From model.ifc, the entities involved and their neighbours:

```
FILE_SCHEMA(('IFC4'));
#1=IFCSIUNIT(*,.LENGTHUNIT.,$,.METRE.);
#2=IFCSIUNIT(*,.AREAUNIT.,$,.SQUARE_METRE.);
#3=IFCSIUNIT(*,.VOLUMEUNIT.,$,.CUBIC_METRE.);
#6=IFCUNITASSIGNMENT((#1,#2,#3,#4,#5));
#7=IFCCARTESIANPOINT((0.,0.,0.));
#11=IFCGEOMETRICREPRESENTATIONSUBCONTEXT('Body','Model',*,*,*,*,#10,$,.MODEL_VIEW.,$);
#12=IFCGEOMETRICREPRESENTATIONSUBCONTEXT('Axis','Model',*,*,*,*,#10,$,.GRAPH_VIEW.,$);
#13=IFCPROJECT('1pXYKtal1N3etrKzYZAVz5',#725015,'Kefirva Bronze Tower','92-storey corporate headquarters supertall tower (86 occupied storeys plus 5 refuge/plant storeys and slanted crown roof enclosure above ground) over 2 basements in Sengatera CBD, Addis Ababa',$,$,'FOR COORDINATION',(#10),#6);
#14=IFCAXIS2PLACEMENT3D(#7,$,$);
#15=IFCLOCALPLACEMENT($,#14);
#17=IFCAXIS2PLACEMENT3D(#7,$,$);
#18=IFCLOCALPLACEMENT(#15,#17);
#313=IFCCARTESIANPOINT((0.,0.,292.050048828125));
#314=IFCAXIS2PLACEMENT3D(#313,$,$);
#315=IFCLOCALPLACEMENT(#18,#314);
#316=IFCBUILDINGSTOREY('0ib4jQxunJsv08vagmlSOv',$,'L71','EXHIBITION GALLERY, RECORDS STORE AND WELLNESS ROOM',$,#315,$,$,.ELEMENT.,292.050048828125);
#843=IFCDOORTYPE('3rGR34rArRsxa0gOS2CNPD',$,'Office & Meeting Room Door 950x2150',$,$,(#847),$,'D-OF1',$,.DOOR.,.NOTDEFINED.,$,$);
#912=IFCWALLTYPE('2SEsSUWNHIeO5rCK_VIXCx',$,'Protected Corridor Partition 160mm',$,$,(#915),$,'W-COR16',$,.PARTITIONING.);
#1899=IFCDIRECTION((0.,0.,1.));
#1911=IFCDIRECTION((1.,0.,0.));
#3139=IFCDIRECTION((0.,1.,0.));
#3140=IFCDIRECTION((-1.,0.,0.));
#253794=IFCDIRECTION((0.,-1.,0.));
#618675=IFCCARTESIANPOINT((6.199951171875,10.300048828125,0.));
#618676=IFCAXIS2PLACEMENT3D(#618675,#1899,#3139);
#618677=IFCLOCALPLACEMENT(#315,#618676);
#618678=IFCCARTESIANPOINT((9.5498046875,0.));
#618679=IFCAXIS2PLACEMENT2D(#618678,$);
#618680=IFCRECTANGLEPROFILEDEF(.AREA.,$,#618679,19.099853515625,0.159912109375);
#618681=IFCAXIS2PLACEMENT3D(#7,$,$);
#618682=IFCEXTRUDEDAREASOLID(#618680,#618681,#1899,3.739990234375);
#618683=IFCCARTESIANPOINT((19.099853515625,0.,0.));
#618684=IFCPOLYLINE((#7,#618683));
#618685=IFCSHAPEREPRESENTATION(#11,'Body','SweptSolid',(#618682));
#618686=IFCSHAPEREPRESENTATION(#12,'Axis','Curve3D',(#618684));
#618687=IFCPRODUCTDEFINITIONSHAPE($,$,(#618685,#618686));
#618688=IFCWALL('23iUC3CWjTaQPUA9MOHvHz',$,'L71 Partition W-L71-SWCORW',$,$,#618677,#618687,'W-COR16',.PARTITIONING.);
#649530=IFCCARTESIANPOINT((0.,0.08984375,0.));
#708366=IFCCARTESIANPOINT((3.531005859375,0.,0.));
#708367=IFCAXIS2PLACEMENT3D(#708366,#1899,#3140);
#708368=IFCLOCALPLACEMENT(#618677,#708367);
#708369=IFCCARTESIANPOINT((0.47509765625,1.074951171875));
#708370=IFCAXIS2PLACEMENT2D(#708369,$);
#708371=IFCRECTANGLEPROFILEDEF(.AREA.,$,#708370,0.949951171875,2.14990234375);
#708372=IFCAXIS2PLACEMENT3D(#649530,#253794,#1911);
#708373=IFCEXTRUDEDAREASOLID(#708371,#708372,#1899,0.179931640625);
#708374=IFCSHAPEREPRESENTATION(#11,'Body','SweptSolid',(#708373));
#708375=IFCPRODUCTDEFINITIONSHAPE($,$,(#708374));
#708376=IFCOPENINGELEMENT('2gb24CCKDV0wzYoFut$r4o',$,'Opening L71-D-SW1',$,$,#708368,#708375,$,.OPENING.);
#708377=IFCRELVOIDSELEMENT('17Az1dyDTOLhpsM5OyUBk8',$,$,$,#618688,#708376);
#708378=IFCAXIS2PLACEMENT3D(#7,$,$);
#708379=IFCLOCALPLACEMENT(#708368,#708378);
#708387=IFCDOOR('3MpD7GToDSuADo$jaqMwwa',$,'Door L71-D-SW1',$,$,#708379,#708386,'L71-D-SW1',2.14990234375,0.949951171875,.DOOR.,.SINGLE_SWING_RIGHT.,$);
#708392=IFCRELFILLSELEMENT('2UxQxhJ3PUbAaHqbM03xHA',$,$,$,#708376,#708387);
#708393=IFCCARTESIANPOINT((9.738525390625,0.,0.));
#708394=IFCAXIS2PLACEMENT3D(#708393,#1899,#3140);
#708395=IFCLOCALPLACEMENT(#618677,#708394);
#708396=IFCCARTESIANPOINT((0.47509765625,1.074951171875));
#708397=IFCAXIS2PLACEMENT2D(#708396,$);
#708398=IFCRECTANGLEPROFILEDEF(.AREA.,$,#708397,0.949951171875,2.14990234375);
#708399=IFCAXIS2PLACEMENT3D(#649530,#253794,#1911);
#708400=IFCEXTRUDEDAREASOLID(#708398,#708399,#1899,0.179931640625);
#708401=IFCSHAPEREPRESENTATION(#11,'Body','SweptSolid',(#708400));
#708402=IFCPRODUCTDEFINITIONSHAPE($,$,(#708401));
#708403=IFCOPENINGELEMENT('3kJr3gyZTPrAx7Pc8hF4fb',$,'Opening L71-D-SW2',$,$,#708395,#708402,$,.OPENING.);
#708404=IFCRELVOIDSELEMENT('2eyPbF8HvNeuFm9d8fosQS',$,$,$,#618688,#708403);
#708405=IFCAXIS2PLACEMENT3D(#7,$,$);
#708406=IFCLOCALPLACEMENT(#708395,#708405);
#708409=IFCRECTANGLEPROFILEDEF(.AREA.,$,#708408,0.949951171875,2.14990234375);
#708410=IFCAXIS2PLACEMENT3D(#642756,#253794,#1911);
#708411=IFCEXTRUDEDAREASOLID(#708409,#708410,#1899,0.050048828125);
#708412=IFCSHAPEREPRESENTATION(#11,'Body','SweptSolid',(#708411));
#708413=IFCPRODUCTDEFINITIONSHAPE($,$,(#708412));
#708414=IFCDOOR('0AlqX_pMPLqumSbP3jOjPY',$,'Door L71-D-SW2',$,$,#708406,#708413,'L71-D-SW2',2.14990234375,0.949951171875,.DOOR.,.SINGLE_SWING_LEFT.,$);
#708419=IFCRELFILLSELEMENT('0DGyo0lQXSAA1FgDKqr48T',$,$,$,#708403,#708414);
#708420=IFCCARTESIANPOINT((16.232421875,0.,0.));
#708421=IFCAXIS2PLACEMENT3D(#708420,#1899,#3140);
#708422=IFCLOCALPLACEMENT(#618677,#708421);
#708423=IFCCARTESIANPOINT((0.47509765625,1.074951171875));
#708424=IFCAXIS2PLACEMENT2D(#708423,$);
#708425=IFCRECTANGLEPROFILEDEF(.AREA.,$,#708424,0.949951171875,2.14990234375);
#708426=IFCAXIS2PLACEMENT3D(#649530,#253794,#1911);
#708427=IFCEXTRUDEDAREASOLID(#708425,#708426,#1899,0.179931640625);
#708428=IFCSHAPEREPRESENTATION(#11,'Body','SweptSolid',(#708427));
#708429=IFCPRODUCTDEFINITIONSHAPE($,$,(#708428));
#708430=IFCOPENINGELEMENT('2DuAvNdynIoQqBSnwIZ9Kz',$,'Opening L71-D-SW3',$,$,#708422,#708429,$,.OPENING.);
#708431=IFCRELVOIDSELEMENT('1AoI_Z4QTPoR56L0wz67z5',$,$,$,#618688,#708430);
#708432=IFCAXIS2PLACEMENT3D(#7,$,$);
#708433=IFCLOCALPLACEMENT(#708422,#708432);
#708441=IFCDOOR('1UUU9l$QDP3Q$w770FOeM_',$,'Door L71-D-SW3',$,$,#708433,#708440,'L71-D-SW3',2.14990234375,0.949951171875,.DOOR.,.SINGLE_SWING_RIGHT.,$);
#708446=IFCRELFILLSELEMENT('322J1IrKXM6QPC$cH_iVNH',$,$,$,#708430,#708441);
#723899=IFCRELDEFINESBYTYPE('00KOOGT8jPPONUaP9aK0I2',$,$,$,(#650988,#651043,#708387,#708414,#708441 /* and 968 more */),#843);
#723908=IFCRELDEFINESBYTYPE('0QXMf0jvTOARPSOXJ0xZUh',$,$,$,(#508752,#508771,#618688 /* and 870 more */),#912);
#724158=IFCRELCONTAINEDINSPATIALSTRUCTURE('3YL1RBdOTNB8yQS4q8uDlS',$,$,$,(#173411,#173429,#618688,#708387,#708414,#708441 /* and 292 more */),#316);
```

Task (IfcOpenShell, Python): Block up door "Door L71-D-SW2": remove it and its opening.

```python
import ifcopenshell
import ifcopenshell.api.feature
import ifcopenshell.api.root
import ifcopenshell.geom
import ifcopenshell.util.shape

model = ifcopenshell.open("model.ifc")
settings = ifcopenshell.geom.settings()


def volume(element):
    """Net volume in cubic metres, openings subtracted."""
    shape = ifcopenshell.geom.create_shape(settings, element)
    return ifcopenshell.util.shape.get_volume(shape.geometry)


door = model.by_id(708414)
opening = door.FillsVoids[0].RelatingOpeningElement
wall = opening.VoidsElements[0].RelatingBuildingElement
before = volume(wall)

ifcopenshell.api.root.remove_product(model, product=door)
ifcopenshell.api.feature.remove_feature(model, feature=opening)

after = volume(wall)

print(f"wall volume {before:.3f} -> {after:.3f} m3")

model.write("model_rev.ifc")
```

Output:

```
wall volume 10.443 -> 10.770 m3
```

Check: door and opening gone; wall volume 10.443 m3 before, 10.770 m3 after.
